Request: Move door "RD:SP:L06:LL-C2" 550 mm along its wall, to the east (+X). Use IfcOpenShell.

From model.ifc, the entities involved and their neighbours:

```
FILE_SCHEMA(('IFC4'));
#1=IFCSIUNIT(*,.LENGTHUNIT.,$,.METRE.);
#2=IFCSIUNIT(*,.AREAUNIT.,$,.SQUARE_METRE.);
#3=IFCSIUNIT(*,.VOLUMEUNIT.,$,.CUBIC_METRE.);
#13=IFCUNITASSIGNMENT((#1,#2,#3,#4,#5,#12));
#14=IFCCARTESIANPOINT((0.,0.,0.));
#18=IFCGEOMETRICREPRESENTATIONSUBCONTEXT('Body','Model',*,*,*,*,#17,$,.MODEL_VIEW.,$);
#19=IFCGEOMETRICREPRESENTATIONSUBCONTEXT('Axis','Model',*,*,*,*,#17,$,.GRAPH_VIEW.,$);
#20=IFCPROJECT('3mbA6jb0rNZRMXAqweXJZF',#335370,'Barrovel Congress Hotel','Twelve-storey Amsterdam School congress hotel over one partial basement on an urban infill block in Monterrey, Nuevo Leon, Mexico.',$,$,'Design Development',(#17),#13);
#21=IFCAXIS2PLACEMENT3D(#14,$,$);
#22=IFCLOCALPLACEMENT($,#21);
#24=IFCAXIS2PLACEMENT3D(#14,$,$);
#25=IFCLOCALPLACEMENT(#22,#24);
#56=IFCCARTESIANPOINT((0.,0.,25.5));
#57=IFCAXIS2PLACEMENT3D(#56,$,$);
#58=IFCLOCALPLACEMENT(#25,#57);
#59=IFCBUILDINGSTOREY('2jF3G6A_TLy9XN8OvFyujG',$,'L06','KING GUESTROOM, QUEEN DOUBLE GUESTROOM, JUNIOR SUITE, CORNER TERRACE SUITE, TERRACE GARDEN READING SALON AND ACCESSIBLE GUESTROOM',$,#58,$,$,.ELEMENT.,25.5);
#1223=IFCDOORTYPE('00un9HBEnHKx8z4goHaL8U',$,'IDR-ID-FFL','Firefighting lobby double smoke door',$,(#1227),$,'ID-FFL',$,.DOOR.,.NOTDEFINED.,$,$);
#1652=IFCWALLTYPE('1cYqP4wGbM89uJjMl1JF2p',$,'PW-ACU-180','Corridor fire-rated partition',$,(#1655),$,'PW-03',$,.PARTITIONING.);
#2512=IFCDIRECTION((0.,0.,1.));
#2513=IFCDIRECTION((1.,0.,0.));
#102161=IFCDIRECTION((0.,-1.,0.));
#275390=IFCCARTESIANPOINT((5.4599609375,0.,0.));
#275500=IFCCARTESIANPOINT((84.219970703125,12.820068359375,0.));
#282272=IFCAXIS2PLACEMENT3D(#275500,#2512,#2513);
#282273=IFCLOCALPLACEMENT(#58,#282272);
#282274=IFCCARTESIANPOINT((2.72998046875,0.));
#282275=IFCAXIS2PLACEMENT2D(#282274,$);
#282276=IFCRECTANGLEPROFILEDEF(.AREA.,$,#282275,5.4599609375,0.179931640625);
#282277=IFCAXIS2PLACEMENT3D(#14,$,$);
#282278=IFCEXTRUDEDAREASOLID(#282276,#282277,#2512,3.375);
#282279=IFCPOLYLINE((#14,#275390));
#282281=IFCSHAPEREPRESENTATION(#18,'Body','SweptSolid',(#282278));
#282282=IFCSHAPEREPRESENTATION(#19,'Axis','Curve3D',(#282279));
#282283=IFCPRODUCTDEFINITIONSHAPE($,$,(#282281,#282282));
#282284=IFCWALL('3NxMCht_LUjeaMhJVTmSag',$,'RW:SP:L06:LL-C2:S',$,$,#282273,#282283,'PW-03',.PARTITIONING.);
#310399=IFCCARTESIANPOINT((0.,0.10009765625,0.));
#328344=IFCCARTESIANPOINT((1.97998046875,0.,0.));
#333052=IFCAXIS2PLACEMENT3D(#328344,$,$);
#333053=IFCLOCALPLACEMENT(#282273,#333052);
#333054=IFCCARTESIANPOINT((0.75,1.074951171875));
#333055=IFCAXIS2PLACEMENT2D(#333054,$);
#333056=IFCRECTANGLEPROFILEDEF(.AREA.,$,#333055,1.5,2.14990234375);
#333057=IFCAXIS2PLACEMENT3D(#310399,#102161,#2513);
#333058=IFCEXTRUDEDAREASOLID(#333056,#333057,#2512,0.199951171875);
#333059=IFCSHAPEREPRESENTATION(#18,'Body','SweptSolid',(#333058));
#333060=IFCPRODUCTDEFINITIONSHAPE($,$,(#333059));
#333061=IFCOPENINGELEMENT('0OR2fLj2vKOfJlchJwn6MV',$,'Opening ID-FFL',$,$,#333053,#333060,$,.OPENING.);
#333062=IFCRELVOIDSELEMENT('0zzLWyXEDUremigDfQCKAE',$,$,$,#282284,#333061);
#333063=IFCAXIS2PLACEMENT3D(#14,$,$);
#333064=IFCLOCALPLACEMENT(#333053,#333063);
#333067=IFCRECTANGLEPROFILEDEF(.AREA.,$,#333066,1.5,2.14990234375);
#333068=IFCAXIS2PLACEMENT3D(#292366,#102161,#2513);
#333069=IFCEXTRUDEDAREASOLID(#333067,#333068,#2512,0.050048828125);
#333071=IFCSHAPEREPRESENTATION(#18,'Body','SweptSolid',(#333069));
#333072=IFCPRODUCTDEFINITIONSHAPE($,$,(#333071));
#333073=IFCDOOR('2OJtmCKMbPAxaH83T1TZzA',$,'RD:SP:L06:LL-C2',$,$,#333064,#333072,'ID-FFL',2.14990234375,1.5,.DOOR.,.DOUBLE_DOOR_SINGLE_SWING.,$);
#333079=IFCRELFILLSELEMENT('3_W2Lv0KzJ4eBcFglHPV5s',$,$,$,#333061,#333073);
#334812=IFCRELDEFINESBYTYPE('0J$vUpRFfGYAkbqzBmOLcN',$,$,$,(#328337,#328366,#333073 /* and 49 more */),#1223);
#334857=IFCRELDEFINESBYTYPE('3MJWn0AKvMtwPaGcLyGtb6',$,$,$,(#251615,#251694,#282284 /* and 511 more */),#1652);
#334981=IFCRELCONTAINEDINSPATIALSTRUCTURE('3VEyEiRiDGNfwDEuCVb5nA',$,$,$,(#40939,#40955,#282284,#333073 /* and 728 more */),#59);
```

```python
import ifcopenshell
import ifcopenshell.api.geometry
import ifcopenshell.util.placement
import ifcopenshell.util.unit

model = ifcopenshell.open("model.ifc")
unit_scale = ifcopenshell.util.unit.calculate_unit_scale(model)

door = model.by_guid("2OJtmCKMbPAxaH83T1TZzA")
opening = door.FillsVoids[0].RelatingOpeningElement
wall = opening.VoidsElements[0].RelatingBuildingElement

wall_matrix = ifcopenshell.util.placement.get_local_placement(wall.ObjectPlacement)
shift = wall_matrix[:3, 0] * 0.55 / unit_scale
before = ifcopenshell.util.placement.get_local_placement(door.ObjectPlacement)[:3, 3].copy()

# The door is placed relative to its opening, so it follows when the opening moves.
matrix = ifcopenshell.util.placement.get_local_placement(opening.ObjectPlacement)
matrix[:3, 3] += shift
ifcopenshell.api.geometry.edit_object_placement(
    model, product=opening, matrix=matrix, is_si=False, should_transform_children=True
)

after = ifcopenshell.util.placement.get_local_placement(door.ObjectPlacement)[:3, 3]
print("door moved by", (after - before).round(3) + 0.0)

model.write("model_v2.ifc")
```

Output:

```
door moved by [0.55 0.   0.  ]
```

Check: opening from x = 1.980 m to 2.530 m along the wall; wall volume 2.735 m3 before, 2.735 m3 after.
